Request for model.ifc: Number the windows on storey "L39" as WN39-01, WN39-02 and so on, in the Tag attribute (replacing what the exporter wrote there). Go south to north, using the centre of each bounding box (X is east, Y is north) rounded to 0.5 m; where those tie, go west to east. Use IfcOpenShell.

First a look at what the model holds.

```python
import ifcopenshell
import ifcopenshell.util.element
import ifcopenshell.util.placement

model = ifcopenshell.open("model.ifc")
print(model.schema)
storey = next(s for s in model.by_type("IfcBuildingStorey") if s.Name == "L39")
windows = [e for e in ifcopenshell.util.element.get_decomposition(storey) if e.is_a("IfcWindow")]
for e in sorted(windows, key=lambda e: e.id()):
    origin = ifcopenshell.util.placement.get_local_placement(e.ObjectPlacement)[:3, 3]
    print(e.id(), e.Tag, e.Name, origin.round(2) + 0.0, sep=" | ")
```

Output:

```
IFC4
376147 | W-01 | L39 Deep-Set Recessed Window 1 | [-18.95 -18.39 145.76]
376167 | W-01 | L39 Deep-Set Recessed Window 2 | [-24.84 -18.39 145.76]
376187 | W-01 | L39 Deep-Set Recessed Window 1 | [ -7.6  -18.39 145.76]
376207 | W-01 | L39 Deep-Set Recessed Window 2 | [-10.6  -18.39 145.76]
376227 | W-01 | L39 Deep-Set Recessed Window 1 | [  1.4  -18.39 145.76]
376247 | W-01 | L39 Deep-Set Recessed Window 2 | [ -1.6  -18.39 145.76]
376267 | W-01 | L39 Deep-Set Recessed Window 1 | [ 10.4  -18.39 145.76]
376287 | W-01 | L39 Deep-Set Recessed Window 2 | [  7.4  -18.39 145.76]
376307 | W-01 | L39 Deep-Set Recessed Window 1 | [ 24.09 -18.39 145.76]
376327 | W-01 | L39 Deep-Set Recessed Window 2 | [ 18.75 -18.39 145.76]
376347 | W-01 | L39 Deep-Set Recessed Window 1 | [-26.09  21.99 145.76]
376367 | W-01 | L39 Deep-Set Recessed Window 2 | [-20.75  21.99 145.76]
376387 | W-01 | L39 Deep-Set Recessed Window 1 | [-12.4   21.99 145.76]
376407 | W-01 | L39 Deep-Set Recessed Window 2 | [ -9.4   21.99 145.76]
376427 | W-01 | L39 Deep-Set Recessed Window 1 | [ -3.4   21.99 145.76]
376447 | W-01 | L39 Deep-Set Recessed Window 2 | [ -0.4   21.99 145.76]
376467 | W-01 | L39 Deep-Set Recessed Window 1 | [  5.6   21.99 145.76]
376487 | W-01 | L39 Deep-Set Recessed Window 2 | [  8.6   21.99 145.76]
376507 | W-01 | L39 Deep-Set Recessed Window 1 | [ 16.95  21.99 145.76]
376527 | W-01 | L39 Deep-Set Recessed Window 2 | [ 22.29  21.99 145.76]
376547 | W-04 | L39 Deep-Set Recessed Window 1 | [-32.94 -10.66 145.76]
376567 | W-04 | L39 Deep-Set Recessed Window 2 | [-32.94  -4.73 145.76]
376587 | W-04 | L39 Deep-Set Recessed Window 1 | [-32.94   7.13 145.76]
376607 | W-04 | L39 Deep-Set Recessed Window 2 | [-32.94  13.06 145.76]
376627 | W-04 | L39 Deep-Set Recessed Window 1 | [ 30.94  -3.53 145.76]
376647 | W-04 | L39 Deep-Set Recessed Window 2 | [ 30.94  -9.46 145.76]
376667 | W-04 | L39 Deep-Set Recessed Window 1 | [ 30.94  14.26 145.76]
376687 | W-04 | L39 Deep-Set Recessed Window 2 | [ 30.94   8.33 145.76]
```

```python
import ifcopenshell
import ifcopenshell.geom
import ifcopenshell.util.element
import ifcopenshell.util.shape

model = ifcopenshell.open("model.ifc")
settings = ifcopenshell.geom.settings()
settings.set("use-world-coords", True)


def centre(element):
    shape = ifcopenshell.geom.create_shape(settings, element)
    return ifcopenshell.util.shape.get_bbox_centroid(shape.geometry)


storey = next(s for s in model.by_type("IfcBuildingStorey") if s.Name == "L39")
windows = [e for e in ifcopenshell.util.element.get_decomposition(storey) if e.is_a("IfcWindow")]

# Insertion points can sit at a corner or the storey origin, so sort by the geometry (in metres).
centres = {e: centre(e) for e in windows}
windows.sort(key=lambda e: (round(centres[e][1] / 0.5), centres[e][0]))

for i, e in enumerate(windows, start=1):
    number = f"WN39-{i:02d}"
    e.Tag = number
    print(e.id(), number)

model.write("model_rev.ifc")
```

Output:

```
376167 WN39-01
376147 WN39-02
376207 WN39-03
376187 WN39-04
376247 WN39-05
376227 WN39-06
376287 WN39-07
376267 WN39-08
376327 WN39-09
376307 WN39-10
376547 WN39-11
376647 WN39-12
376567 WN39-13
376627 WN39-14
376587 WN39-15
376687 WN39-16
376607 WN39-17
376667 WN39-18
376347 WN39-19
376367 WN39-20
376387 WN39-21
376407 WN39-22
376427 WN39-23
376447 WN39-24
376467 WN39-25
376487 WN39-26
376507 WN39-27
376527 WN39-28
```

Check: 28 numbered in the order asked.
